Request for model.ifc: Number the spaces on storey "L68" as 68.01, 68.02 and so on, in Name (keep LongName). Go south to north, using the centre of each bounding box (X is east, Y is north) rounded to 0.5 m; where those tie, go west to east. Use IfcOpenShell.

First a look at what the model holds.

```python
import ifcopenshell
import ifcopenshell.util.element
import ifcopenshell.util.placement

model = ifcopenshell.open("model.ifc")
print(model.schema)
storey = next(s for s in model.by_type("IfcBuildingStorey") if s.Name == "L68")
spaces = [e for e in ifcopenshell.util.element.get_decomposition(storey) if e.is_a("IfcSpace")]
for e in sorted(spaces, key=lambda e: e.id()):
    origin = ifcopenshell.util.placement.get_local_placement(e.ObjectPlacement)[:3, 3]
    print(e.id(), e.Name, e.LongName, origin.round(2) + 0.0, sep=" | ")
```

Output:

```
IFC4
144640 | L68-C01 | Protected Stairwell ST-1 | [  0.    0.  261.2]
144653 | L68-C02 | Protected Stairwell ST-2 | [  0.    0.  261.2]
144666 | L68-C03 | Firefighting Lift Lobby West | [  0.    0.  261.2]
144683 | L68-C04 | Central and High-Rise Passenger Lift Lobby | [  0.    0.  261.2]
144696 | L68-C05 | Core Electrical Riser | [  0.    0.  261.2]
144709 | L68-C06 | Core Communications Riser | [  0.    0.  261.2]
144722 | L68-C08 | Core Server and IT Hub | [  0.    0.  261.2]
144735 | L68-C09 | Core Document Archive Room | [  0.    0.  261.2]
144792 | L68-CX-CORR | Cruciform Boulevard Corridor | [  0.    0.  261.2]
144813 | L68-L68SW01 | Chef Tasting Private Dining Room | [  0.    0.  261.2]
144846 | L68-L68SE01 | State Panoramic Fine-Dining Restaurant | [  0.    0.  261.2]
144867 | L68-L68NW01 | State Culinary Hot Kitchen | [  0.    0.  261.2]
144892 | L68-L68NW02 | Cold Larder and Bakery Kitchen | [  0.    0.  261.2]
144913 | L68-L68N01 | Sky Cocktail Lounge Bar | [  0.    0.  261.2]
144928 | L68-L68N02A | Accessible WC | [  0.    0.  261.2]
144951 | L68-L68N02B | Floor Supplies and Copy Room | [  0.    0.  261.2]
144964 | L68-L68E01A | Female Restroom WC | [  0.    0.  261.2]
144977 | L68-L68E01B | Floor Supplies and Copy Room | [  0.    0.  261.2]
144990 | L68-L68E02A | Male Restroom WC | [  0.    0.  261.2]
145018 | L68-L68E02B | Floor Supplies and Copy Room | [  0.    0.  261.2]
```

```python
import ifcopenshell
import ifcopenshell.geom
import ifcopenshell.util.element
import ifcopenshell.util.shape

model = ifcopenshell.open("model.ifc")
settings = ifcopenshell.geom.settings()
settings.set("use-world-coords", True)


def centre(element):
    shape = ifcopenshell.geom.create_shape(settings, element)
    return ifcopenshell.util.shape.get_bbox_centroid(shape.geometry)


storey = next(s for s in model.by_type("IfcBuildingStorey") if s.Name == "L68")
spaces = [e for e in ifcopenshell.util.element.get_decomposition(storey) if e.is_a("IfcSpace")]

# Insertion points can sit at a corner or the storey origin, so sort by the geometry (in metres).
centres = {e: centre(e) for e in spaces}
spaces.sort(key=lambda e: (round(centres[e][1] / 0.5), centres[e][0]))

for i, e in enumerate(spaces, start=1):
    number = f"68.{i:02d}"
    e.Name = number
    print(e.id(), number)

model.write("model_updated.ifc")
```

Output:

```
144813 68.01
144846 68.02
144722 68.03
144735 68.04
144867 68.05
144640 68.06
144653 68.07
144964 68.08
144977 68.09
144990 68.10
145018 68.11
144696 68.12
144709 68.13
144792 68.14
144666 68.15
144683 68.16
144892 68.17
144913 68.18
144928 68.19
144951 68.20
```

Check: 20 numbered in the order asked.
